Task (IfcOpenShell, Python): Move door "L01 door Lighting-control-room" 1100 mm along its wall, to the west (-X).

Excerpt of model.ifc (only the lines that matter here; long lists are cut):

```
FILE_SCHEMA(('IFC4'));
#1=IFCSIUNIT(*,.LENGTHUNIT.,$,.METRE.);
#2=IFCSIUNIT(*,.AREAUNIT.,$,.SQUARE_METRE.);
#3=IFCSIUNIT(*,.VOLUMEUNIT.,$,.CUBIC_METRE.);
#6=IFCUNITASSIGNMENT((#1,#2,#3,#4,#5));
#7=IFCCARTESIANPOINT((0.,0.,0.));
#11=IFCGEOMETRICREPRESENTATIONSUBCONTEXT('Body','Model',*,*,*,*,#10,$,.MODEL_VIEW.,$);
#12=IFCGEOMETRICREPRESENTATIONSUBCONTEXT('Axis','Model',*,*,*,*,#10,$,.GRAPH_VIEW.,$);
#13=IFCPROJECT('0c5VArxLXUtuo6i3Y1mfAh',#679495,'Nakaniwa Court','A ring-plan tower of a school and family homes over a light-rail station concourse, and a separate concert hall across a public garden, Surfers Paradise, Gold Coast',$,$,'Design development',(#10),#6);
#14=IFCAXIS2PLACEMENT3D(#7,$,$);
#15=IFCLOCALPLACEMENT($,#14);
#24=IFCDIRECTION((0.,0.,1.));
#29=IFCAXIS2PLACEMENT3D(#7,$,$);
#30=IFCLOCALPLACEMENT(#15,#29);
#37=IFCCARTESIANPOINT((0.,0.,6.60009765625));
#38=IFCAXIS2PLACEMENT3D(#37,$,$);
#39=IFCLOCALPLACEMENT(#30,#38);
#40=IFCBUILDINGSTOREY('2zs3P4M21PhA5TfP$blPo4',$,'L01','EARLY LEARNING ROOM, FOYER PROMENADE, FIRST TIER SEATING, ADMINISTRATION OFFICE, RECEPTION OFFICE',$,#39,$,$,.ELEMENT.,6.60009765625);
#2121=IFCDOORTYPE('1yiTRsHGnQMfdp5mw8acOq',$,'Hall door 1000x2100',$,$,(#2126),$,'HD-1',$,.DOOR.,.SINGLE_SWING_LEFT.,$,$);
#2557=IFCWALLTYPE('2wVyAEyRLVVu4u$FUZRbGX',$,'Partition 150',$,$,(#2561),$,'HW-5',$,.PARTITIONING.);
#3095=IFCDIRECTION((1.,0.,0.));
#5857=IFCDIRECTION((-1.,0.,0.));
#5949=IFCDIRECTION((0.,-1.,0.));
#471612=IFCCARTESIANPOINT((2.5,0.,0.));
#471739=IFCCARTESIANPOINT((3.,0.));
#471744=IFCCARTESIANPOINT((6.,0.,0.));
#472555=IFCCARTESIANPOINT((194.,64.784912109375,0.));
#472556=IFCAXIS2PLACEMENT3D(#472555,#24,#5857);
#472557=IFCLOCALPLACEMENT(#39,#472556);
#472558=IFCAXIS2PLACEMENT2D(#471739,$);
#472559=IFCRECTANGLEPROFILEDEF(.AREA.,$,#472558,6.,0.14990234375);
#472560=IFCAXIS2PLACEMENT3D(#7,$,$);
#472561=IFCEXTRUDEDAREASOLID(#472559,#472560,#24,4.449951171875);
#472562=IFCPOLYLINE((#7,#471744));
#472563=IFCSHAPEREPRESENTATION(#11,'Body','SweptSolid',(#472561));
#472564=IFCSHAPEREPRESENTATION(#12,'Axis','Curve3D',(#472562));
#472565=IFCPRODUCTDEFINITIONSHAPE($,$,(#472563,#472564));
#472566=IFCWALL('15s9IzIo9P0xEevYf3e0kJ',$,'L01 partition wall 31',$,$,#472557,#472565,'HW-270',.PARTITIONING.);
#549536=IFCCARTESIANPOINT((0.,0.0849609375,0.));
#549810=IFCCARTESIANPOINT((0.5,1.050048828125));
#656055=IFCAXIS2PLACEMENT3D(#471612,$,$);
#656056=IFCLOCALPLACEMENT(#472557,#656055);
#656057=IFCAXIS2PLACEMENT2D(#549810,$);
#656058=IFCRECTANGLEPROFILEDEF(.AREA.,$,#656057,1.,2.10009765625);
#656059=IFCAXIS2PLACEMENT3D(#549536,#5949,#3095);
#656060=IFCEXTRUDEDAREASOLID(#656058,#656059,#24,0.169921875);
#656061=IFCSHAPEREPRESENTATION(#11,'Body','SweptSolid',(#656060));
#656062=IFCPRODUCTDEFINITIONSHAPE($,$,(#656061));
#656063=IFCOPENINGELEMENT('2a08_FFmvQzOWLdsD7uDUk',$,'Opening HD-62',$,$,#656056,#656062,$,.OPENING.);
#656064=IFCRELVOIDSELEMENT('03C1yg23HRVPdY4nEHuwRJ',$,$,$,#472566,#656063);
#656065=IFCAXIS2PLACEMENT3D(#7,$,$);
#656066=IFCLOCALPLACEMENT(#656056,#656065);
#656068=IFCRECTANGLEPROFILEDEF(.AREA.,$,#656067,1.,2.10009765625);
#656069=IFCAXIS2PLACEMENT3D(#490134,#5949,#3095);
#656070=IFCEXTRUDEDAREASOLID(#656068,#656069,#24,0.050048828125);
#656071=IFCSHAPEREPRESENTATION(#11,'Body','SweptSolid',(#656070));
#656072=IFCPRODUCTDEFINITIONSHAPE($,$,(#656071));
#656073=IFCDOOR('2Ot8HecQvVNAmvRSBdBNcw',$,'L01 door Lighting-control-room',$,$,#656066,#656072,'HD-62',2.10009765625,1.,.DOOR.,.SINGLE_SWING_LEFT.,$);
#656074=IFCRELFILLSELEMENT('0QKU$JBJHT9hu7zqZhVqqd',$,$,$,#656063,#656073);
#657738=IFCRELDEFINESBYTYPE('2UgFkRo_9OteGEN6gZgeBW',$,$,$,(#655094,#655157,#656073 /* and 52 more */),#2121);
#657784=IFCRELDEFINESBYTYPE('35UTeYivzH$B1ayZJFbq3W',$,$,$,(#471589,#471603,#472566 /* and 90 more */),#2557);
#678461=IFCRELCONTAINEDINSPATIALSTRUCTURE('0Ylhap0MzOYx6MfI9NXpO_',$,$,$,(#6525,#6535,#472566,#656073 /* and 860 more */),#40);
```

```python
import ifcopenshell
import ifcopenshell.api.geometry
import ifcopenshell.util.placement
import ifcopenshell.util.unit

model = ifcopenshell.open("model.ifc")
unit_scale = ifcopenshell.util.unit.calculate_unit_scale(model)

door = model.by_guid("2Ot8HecQvVNAmvRSBdBNcw")
opening = door.FillsVoids[0].RelatingOpeningElement
wall = opening.VoidsElements[0].RelatingBuildingElement

wall_matrix = ifcopenshell.util.placement.get_local_placement(wall.ObjectPlacement)
shift = wall_matrix[:3, 0] * 1.1 / unit_scale
before = ifcopenshell.util.placement.get_local_placement(door.ObjectPlacement)[:3, 3].copy()

# The door is placed relative to its opening, so it follows when the opening moves.
matrix = ifcopenshell.util.placement.get_local_placement(opening.ObjectPlacement)
matrix[:3, 3] += shift
ifcopenshell.api.geometry.edit_object_placement(
    model, product=opening, matrix=matrix, is_si=False, should_transform_children=True
)

after = ifcopenshell.util.placement.get_local_placement(door.ObjectPlacement)[:3, 3]
print("door moved by", (after - before).round(3) + 0.0)

model.write("model-out.ifc")
```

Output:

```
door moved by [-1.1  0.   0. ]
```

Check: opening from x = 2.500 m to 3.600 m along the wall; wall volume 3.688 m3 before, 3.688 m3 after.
